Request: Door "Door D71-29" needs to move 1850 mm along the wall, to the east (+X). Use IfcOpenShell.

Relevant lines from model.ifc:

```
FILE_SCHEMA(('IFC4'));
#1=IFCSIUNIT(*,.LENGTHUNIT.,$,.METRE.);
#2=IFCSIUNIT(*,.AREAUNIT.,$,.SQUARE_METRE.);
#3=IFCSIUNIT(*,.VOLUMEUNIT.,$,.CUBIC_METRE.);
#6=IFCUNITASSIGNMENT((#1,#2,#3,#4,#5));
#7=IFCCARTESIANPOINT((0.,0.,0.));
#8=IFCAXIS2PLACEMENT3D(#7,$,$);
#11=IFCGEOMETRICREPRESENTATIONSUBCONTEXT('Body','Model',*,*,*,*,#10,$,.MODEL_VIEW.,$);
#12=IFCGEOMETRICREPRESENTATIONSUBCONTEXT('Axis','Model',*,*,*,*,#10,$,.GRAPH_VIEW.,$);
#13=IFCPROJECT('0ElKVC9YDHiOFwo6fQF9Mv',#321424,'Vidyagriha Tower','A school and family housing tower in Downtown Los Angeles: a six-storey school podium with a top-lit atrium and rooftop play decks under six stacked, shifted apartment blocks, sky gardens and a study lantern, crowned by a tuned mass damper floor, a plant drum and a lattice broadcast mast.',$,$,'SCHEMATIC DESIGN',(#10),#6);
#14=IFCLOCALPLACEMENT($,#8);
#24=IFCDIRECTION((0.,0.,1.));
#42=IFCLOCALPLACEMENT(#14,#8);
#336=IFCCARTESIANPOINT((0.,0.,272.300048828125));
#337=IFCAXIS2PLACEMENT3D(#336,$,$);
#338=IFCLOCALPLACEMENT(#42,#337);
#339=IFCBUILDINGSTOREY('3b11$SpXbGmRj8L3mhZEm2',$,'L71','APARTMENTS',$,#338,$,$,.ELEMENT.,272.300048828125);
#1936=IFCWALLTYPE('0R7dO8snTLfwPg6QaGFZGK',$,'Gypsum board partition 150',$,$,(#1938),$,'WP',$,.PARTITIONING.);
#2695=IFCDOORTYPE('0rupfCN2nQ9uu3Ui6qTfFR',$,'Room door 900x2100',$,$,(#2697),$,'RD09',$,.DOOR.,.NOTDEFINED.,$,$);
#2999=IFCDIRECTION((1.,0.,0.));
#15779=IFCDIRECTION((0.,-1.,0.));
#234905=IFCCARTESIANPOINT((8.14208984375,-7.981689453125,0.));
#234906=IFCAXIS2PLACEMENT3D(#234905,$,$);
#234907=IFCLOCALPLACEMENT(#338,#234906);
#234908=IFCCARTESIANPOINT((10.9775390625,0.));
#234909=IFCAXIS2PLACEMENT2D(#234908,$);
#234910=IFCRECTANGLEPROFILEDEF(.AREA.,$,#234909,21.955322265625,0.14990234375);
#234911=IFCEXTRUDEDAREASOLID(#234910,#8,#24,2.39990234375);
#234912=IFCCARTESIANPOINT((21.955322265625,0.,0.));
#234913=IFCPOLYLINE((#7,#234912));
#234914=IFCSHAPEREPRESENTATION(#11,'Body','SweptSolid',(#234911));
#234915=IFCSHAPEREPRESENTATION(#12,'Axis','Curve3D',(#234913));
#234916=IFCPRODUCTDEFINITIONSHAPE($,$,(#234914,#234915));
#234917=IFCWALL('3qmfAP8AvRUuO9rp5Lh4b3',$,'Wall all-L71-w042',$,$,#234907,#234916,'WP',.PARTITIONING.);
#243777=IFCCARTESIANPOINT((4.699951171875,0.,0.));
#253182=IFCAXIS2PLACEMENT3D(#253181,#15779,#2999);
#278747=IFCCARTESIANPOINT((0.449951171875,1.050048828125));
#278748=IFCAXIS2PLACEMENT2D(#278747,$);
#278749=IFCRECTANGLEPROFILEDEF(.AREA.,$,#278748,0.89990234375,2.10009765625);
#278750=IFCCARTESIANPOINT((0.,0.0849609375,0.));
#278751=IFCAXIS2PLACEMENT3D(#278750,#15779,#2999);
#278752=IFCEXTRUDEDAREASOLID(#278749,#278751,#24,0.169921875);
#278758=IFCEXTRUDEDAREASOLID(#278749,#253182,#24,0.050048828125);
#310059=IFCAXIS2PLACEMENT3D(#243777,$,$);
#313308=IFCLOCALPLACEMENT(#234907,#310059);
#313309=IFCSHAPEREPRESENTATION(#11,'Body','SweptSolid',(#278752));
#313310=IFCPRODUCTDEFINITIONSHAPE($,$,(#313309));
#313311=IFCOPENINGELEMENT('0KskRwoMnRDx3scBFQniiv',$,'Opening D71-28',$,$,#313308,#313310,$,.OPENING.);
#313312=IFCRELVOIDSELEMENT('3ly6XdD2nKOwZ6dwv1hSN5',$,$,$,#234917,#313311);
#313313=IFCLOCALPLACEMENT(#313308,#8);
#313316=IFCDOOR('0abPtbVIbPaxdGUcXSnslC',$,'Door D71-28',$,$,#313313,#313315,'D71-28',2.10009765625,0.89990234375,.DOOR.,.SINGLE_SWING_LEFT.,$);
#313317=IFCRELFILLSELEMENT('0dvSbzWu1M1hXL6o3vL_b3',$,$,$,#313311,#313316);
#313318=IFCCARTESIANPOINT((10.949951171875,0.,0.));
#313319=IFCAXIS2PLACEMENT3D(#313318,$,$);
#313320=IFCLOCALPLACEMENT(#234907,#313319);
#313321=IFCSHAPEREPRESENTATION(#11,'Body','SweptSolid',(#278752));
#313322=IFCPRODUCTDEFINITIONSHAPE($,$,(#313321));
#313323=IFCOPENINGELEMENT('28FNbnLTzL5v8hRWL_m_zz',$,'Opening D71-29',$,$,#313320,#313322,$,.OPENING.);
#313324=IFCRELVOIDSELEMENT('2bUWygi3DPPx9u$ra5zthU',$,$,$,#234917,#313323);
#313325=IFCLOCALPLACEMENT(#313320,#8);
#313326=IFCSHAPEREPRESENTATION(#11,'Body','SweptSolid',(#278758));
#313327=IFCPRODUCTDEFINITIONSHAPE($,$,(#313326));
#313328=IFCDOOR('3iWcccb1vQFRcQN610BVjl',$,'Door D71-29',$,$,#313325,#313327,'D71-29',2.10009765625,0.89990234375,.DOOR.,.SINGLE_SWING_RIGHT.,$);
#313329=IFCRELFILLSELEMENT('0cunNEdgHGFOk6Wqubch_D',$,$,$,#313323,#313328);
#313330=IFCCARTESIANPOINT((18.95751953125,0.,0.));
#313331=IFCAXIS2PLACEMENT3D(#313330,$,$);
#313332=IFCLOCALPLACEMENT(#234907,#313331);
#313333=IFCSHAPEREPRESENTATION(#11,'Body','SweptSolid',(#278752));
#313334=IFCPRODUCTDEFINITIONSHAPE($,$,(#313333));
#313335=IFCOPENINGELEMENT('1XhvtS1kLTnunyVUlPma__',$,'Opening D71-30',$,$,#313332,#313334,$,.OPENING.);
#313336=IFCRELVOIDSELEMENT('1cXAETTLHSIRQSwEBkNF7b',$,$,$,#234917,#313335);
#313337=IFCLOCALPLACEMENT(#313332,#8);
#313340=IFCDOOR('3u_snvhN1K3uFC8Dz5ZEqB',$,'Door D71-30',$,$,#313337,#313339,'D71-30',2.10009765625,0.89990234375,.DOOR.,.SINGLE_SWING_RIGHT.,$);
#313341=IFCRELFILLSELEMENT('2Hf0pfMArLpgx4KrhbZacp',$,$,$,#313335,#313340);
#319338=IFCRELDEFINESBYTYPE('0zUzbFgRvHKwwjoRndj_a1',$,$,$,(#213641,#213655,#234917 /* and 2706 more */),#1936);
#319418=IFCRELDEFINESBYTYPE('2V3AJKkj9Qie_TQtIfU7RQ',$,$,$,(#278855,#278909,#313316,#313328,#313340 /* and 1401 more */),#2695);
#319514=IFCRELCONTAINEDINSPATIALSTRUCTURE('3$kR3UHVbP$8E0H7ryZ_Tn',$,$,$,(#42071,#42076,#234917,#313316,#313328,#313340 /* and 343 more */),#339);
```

```python
import ifcopenshell
import ifcopenshell.api.geometry
import ifcopenshell.util.placement
import ifcopenshell.util.unit

model = ifcopenshell.open("model.ifc")
unit_scale = ifcopenshell.util.unit.calculate_unit_scale(model)

door = model.by_guid("3iWcccb1vQFRcQN610BVjl")
opening = door.FillsVoids[0].RelatingOpeningElement
wall = opening.VoidsElements[0].RelatingBuildingElement

wall_matrix = ifcopenshell.util.placement.get_local_placement(wall.ObjectPlacement)
shift = wall_matrix[:3, 0] * 1.85 / unit_scale
before = ifcopenshell.util.placement.get_local_placement(door.ObjectPlacement)[:3, 3].copy()

# The door is placed relative to its opening, so it follows when the opening moves.
matrix = ifcopenshell.util.placement.get_local_placement(opening.ObjectPlacement)
matrix[:3, 3] += shift
ifcopenshell.api.geometry.edit_object_placement(
    model, product=opening, matrix=matrix, is_si=False, should_transform_children=True
)

after = ifcopenshell.util.placement.get_local_placement(door.ObjectPlacement)[:3, 3]
print("door moved by", (after - before).round(3) + 0.0)

model.write("model_updated.ifc")
```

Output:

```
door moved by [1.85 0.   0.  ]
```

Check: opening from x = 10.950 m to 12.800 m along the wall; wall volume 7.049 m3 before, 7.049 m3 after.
